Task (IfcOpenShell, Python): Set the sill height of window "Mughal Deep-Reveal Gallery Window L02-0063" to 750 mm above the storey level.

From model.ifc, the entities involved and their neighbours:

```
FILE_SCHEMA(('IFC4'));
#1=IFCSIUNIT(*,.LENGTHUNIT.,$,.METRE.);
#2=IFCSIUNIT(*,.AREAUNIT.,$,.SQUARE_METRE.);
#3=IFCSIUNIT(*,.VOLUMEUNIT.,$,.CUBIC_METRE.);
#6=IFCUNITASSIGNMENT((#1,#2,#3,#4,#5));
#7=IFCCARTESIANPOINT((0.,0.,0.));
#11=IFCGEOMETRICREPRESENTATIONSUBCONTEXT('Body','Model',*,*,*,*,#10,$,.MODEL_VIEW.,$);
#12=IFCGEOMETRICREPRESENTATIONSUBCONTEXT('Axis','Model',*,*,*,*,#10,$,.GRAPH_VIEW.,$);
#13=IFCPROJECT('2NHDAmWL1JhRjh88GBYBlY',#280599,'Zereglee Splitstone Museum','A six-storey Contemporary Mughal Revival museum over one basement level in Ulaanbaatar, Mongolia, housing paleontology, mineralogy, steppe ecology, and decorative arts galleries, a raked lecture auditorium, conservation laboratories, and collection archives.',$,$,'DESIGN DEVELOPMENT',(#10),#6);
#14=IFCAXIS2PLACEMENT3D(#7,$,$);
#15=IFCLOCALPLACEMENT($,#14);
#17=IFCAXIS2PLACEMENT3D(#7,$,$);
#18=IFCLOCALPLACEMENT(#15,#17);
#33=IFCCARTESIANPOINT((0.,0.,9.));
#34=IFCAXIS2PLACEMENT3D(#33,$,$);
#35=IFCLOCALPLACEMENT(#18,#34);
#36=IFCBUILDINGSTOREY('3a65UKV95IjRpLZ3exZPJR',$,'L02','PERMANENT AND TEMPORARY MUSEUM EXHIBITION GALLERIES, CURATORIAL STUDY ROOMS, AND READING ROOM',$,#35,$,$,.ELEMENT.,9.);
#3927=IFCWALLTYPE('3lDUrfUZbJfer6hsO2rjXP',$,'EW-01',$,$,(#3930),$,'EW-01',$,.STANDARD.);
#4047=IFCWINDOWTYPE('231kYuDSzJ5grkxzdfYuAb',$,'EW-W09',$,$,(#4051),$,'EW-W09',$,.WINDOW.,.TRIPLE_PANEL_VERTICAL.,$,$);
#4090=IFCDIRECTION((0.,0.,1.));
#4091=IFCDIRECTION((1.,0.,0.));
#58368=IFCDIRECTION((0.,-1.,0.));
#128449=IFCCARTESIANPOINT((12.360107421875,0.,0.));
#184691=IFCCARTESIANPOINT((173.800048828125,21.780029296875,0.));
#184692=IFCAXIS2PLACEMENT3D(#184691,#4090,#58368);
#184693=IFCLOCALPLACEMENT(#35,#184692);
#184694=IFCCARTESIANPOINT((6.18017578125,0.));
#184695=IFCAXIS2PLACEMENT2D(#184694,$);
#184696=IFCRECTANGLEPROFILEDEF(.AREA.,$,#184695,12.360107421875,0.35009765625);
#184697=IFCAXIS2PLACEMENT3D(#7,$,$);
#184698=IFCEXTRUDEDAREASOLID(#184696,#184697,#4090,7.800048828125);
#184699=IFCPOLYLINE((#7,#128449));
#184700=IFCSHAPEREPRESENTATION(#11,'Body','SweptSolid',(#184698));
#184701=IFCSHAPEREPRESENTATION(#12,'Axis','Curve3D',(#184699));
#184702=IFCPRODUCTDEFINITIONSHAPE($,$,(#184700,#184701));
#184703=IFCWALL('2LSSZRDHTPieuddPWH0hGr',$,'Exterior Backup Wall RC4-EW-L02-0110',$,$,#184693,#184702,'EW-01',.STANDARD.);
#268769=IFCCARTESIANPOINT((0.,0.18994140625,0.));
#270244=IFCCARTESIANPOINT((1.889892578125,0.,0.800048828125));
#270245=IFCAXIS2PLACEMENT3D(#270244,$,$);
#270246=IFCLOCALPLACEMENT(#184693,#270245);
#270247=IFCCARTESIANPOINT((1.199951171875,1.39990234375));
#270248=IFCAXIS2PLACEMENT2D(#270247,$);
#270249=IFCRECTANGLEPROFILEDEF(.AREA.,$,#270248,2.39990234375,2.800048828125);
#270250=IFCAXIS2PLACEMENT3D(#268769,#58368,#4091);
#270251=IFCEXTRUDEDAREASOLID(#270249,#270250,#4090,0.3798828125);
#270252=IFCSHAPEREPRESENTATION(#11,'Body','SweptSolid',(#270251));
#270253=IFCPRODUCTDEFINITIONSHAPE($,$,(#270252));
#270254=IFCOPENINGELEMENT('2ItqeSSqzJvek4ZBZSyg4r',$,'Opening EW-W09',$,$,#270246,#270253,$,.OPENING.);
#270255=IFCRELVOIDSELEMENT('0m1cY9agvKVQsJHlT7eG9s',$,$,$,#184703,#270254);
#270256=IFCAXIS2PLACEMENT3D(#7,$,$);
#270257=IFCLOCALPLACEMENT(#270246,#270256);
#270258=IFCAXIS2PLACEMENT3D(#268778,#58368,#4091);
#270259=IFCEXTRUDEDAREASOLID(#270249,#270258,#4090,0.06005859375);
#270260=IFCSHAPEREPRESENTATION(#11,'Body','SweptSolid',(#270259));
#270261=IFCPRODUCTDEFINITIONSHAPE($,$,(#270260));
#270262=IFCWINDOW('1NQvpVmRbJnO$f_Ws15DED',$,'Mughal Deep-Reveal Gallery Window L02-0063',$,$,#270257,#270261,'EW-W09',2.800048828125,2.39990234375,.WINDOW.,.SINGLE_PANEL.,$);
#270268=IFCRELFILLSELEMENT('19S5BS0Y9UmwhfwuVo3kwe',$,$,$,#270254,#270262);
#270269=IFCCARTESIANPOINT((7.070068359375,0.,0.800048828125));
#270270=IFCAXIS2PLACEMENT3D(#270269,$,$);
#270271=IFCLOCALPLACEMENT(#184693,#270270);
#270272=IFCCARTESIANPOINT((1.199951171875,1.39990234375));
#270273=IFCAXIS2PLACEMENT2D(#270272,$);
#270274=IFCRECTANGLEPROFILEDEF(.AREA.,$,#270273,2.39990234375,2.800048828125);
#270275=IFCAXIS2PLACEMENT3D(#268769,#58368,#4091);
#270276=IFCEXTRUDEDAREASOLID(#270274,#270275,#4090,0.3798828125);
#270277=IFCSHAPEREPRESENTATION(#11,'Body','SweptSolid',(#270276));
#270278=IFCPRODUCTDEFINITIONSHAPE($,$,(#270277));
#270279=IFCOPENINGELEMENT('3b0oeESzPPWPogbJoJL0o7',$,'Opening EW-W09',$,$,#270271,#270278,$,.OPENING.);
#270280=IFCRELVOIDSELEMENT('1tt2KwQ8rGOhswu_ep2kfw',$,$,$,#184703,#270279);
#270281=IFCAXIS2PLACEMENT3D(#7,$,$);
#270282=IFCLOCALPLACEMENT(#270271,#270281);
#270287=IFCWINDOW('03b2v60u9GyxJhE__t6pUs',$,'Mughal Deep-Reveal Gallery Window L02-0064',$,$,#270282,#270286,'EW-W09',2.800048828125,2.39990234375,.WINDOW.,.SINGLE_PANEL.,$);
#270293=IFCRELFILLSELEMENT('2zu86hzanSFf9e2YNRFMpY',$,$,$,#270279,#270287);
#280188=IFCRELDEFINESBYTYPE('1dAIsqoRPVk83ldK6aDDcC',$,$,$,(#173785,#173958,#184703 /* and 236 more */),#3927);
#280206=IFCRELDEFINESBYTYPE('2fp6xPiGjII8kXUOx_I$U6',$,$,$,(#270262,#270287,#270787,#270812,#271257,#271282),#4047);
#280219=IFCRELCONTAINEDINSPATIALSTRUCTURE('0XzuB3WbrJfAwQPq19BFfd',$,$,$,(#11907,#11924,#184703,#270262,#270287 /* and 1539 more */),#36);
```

```python
import numpy as np
import ifcopenshell
import ifcopenshell.api.geometry
import ifcopenshell.geom
import ifcopenshell.util.element
import ifcopenshell.util.placement
import ifcopenshell.util.shape
import ifcopenshell.util.unit

model = ifcopenshell.open("model.ifc")
unit_scale = ifcopenshell.util.unit.calculate_unit_scale(model)

window = model.by_guid("1NQvpVmRbJnO$f_Ws15DED")
opening = window.FillsVoids[0].RelatingOpeningElement
storey = ifcopenshell.util.element.get_container(window, ifc_class="IfcBuildingStorey")
level = ifcopenshell.util.placement.get_local_placement(storey.ObjectPlacement)[2, 3]

# The opening's origin need not be at the sill, so measure its lowest point.
shape = ifcopenshell.geom.create_shape(ifcopenshell.geom.settings(), opening)
bottom = ifcopenshell.util.shape.get_shape_bottom_elevation(shape, shape.geometry) / unit_scale
dz = level + 0.75 / unit_scale - bottom

shift = np.array([0.0, 0.0, dz])
# The window is placed relative to its opening, so it follows when the opening moves.
matrix = ifcopenshell.util.placement.get_local_placement(opening.ObjectPlacement)
matrix[:3, 3] += shift
ifcopenshell.api.geometry.edit_object_placement(
    model, product=opening, matrix=matrix, is_si=False, should_transform_children=True
)

print(f"moved by {dz * unit_scale:+.3f} m")

model.write("model-out.ifc")
```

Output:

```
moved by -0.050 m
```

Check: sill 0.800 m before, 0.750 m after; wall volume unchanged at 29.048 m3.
